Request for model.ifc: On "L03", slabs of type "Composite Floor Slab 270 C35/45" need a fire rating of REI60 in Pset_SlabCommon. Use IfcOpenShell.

First a look at what the model holds.

```python
import ifcopenshell
import ifcopenshell.util.element

model = ifcopenshell.open("model.ifc")
print(model.schema)
storey = next(s for s in model.by_type("IfcBuildingStorey") if s.Name == "L03")
slabs = [e for e in ifcopenshell.util.element.get_decomposition(storey) if e.is_a("IfcSlab")]
seen = {}
for e in slabs:
    element_type = ifcopenshell.util.element.get_type(e)
    key = (element_type.Name if element_type != e and element_type else None, ifcopenshell.util.element.get_pset(e, "Pset_SlabCommon", "FireRating"))
    seen[key] = seen.get(key, 0) + 1
for (name, value), count in sorted(seen.items(), key=str):
    print(count, "x", name, "|", value)
```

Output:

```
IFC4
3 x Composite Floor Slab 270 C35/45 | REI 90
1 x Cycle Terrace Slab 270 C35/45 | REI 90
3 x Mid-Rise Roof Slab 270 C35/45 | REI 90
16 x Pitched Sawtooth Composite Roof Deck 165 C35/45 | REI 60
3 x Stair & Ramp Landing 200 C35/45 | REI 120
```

```python
import ifcopenshell
import ifcopenshell.api.pset
import ifcopenshell.util.element

model = ifcopenshell.open("model.ifc")

storey = next(s for s in model.by_type("IfcBuildingStorey") if s.Name == "L03")
slabs = [e for e in ifcopenshell.util.element.get_decomposition(storey) if e.is_a("IfcSlab")]

count = 0
for e in slabs:
    element_type = ifcopenshell.util.element.get_type(e)
    if element_type in (None, e) or element_type.Name != "Composite Floor Slab 270 C35/45":
        continue
    # add_pset returns the element's existing set when there is one.
    pset = ifcopenshell.api.pset.add_pset(model, product=e, name="Pset_SlabCommon")
    ifcopenshell.api.pset.edit_pset(model, pset=pset, properties={"FireRating": "REI60"})
    count += 1

print(count, "slabs updated")

model.write("model_rev.ifc")
```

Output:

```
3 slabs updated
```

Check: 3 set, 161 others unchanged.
